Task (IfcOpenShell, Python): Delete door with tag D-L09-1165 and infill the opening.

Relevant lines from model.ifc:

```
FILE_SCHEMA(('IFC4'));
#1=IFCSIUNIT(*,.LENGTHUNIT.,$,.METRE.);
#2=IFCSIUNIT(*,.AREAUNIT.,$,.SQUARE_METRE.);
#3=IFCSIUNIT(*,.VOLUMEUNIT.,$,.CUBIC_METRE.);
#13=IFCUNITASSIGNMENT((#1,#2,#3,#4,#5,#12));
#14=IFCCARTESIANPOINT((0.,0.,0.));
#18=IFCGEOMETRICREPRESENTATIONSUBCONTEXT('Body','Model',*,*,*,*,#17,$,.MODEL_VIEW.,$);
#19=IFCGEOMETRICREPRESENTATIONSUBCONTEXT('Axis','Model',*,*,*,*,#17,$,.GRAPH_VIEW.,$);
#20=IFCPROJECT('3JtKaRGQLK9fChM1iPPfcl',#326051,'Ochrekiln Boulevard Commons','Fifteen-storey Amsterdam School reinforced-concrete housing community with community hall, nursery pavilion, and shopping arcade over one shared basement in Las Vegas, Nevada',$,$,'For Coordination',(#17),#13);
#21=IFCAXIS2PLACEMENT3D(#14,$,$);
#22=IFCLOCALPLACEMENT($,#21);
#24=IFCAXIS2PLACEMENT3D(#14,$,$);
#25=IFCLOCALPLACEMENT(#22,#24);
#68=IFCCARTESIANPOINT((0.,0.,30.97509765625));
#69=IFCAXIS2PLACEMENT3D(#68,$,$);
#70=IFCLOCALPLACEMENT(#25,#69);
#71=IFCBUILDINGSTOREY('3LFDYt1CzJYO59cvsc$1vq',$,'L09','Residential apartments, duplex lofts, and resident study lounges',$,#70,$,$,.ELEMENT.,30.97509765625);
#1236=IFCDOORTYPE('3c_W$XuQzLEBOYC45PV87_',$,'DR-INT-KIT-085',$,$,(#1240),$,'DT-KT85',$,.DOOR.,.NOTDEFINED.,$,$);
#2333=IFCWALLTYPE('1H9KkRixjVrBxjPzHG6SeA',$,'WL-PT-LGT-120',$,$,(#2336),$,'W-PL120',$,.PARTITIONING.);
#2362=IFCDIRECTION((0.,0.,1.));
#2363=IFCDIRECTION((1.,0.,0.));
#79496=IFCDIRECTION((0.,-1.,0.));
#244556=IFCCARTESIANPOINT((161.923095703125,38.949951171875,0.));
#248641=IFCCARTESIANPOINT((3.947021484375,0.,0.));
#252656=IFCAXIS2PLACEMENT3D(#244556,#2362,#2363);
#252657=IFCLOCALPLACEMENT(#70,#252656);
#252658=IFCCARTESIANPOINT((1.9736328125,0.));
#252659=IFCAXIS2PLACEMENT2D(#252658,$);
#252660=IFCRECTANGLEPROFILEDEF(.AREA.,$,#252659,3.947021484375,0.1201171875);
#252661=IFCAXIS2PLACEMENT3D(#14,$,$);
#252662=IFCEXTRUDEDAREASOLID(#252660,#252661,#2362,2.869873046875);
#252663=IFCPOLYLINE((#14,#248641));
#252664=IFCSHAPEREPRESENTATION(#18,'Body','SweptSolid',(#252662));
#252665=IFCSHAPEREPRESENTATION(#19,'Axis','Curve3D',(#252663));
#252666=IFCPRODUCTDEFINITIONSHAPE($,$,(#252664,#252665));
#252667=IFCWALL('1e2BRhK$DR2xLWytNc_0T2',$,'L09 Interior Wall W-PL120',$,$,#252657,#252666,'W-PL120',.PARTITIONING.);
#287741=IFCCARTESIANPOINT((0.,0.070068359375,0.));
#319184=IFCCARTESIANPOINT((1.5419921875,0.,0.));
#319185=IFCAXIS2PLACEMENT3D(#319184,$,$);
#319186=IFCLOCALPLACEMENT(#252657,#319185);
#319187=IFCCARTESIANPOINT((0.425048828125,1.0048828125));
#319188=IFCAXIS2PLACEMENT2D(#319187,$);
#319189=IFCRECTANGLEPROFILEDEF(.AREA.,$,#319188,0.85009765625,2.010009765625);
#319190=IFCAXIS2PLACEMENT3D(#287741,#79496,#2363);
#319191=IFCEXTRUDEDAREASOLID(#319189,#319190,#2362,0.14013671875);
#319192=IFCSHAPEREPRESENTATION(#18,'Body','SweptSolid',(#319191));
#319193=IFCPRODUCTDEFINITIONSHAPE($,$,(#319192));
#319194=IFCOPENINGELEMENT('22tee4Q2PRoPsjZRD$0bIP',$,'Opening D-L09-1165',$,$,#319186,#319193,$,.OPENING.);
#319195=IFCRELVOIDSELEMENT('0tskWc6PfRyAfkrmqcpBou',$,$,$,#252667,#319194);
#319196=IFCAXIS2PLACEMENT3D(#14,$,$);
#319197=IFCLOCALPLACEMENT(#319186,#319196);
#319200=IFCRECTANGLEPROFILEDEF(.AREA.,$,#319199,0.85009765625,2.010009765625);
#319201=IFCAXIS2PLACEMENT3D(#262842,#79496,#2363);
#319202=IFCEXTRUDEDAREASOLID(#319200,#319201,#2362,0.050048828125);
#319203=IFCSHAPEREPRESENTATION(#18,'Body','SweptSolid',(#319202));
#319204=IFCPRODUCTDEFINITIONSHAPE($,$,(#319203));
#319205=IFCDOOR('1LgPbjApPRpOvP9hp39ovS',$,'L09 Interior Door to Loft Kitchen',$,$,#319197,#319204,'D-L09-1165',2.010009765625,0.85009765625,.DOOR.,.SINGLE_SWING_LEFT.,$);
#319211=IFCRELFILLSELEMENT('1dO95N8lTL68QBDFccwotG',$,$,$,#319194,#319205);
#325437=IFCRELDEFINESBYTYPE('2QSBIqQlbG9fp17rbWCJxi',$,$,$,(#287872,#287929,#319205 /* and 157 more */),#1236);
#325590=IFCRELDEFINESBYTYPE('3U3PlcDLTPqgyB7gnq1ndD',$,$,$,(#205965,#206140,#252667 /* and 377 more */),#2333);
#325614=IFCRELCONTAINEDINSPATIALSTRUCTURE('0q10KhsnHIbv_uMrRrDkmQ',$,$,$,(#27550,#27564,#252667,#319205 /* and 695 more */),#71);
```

```python
import ifcopenshell
import ifcopenshell.api.feature
import ifcopenshell.api.root
import ifcopenshell.geom
import ifcopenshell.util.shape

model = ifcopenshell.open("model.ifc")
settings = ifcopenshell.geom.settings()


def volume(element):
    """Net volume in cubic metres, openings subtracted."""
    shape = ifcopenshell.geom.create_shape(settings, element)
    return ifcopenshell.util.shape.get_volume(shape.geometry)


door = model.by_id(319205)
opening = door.FillsVoids[0].RelatingOpeningElement
wall = opening.VoidsElements[0].RelatingBuildingElement
before = volume(wall)

ifcopenshell.api.root.remove_product(model, product=door)
ifcopenshell.api.feature.remove_feature(model, feature=opening)

after = volume(wall)

print(f"wall volume {before:.3f} -> {after:.3f} m3")

model.write("model-out.ifc")
```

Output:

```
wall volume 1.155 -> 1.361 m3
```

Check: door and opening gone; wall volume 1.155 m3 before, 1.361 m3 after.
